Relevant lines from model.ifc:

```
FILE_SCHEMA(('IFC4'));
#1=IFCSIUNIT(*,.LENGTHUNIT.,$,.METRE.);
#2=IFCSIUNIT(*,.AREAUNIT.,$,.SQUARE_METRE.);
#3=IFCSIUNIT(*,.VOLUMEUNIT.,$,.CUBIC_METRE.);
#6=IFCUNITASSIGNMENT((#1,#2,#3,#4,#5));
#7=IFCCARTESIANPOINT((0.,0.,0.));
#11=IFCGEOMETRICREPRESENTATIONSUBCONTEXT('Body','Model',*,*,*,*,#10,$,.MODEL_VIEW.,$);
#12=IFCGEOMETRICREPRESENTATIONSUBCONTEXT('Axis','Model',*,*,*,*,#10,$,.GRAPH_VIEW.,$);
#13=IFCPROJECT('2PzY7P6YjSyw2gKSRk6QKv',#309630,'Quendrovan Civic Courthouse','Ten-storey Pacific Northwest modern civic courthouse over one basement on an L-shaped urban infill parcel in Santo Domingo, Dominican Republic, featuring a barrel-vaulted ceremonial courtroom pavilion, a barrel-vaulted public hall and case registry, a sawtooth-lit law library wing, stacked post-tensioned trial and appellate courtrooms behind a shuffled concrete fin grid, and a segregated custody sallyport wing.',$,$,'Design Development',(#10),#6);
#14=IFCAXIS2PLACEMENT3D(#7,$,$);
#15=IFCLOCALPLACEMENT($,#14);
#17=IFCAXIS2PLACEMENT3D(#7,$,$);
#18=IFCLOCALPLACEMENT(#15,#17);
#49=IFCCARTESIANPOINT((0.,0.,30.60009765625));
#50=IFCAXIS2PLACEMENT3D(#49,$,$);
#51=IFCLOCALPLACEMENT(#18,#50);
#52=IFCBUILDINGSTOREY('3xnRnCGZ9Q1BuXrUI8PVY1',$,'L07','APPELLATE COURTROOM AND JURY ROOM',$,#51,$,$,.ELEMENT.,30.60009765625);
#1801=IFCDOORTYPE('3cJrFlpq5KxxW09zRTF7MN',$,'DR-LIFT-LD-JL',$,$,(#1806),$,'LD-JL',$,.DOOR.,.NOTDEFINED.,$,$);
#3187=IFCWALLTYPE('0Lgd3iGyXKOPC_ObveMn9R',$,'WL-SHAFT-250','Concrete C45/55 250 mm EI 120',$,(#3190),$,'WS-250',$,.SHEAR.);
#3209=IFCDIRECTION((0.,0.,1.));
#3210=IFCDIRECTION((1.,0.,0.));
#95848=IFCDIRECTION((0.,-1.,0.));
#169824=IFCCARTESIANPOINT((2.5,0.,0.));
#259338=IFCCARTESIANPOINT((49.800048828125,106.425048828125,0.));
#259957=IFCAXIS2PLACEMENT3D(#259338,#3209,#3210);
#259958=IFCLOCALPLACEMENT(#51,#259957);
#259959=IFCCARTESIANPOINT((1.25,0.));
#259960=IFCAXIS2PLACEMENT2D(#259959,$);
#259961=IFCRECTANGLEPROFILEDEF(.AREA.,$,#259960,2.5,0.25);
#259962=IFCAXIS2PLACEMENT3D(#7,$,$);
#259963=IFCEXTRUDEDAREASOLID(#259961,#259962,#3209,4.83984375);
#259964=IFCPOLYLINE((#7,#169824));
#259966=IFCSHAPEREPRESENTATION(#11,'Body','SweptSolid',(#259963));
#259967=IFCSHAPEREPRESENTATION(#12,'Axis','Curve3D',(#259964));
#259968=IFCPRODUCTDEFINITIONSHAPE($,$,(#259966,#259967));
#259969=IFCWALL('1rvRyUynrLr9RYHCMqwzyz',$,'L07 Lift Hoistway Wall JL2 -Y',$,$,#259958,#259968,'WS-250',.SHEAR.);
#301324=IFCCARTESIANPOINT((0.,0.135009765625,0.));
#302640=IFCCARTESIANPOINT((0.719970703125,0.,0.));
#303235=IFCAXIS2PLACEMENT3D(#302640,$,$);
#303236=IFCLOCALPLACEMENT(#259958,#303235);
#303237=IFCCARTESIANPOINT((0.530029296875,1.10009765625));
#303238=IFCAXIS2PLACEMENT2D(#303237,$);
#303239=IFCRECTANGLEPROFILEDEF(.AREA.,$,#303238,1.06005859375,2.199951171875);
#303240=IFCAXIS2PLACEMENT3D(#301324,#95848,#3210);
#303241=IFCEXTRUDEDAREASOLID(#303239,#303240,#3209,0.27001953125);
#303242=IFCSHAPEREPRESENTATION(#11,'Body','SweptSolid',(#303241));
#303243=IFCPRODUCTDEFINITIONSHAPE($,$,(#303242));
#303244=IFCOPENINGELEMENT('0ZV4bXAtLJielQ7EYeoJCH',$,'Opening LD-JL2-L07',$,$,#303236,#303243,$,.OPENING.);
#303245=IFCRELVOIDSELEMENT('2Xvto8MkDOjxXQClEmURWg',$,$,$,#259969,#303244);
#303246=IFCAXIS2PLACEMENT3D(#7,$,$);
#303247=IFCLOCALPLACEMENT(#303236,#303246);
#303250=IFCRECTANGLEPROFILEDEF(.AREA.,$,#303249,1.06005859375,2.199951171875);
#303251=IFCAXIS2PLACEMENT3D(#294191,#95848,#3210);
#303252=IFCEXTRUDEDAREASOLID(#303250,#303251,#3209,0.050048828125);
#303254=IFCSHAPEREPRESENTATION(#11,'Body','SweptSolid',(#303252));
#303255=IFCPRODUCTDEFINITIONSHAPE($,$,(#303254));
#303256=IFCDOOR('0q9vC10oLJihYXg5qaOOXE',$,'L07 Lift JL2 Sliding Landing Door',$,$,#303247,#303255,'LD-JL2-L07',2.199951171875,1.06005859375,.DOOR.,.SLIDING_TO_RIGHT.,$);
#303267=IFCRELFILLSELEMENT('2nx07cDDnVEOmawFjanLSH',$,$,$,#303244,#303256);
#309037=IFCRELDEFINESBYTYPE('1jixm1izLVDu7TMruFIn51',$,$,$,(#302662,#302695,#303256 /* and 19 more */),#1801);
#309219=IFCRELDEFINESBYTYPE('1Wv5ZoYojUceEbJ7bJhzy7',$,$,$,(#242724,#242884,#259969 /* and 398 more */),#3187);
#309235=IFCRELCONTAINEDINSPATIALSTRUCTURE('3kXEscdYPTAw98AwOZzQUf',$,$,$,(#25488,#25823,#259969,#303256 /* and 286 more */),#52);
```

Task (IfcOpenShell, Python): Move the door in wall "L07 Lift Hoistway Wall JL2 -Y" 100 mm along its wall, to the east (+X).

```python
import ifcopenshell
import ifcopenshell.api.geometry
import ifcopenshell.util.placement

model = ifcopenshell.open("model.ifc")

door = model.by_guid("0q9vC10oLJihYXg5qaOOXE")
opening = door.FillsVoids[0].RelatingOpeningElement
wall = opening.VoidsElements[0].RelatingBuildingElement

wall_matrix = ifcopenshell.util.placement.get_local_placement(wall.ObjectPlacement)
shift = wall_matrix[:3, 0] * 0.1
before = ifcopenshell.util.placement.get_local_placement(door.ObjectPlacement)[:3, 3].copy()

# The door is placed relative to its opening, so it follows when the opening moves.
matrix = ifcopenshell.util.placement.get_local_placement(opening.ObjectPlacement)
matrix[:3, 3] += shift
ifcopenshell.api.geometry.edit_object_placement(
    model, product=opening, matrix=matrix, is_si=False, should_transform_children=True
)

after = ifcopenshell.util.placement.get_local_placement(door.ObjectPlacement)[:3, 3]
print("door moved by", (after - before).round(3) + 0.0)

model.write("model_updated.ifc")
```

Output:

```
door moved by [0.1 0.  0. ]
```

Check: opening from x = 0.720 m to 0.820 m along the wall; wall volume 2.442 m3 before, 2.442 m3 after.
